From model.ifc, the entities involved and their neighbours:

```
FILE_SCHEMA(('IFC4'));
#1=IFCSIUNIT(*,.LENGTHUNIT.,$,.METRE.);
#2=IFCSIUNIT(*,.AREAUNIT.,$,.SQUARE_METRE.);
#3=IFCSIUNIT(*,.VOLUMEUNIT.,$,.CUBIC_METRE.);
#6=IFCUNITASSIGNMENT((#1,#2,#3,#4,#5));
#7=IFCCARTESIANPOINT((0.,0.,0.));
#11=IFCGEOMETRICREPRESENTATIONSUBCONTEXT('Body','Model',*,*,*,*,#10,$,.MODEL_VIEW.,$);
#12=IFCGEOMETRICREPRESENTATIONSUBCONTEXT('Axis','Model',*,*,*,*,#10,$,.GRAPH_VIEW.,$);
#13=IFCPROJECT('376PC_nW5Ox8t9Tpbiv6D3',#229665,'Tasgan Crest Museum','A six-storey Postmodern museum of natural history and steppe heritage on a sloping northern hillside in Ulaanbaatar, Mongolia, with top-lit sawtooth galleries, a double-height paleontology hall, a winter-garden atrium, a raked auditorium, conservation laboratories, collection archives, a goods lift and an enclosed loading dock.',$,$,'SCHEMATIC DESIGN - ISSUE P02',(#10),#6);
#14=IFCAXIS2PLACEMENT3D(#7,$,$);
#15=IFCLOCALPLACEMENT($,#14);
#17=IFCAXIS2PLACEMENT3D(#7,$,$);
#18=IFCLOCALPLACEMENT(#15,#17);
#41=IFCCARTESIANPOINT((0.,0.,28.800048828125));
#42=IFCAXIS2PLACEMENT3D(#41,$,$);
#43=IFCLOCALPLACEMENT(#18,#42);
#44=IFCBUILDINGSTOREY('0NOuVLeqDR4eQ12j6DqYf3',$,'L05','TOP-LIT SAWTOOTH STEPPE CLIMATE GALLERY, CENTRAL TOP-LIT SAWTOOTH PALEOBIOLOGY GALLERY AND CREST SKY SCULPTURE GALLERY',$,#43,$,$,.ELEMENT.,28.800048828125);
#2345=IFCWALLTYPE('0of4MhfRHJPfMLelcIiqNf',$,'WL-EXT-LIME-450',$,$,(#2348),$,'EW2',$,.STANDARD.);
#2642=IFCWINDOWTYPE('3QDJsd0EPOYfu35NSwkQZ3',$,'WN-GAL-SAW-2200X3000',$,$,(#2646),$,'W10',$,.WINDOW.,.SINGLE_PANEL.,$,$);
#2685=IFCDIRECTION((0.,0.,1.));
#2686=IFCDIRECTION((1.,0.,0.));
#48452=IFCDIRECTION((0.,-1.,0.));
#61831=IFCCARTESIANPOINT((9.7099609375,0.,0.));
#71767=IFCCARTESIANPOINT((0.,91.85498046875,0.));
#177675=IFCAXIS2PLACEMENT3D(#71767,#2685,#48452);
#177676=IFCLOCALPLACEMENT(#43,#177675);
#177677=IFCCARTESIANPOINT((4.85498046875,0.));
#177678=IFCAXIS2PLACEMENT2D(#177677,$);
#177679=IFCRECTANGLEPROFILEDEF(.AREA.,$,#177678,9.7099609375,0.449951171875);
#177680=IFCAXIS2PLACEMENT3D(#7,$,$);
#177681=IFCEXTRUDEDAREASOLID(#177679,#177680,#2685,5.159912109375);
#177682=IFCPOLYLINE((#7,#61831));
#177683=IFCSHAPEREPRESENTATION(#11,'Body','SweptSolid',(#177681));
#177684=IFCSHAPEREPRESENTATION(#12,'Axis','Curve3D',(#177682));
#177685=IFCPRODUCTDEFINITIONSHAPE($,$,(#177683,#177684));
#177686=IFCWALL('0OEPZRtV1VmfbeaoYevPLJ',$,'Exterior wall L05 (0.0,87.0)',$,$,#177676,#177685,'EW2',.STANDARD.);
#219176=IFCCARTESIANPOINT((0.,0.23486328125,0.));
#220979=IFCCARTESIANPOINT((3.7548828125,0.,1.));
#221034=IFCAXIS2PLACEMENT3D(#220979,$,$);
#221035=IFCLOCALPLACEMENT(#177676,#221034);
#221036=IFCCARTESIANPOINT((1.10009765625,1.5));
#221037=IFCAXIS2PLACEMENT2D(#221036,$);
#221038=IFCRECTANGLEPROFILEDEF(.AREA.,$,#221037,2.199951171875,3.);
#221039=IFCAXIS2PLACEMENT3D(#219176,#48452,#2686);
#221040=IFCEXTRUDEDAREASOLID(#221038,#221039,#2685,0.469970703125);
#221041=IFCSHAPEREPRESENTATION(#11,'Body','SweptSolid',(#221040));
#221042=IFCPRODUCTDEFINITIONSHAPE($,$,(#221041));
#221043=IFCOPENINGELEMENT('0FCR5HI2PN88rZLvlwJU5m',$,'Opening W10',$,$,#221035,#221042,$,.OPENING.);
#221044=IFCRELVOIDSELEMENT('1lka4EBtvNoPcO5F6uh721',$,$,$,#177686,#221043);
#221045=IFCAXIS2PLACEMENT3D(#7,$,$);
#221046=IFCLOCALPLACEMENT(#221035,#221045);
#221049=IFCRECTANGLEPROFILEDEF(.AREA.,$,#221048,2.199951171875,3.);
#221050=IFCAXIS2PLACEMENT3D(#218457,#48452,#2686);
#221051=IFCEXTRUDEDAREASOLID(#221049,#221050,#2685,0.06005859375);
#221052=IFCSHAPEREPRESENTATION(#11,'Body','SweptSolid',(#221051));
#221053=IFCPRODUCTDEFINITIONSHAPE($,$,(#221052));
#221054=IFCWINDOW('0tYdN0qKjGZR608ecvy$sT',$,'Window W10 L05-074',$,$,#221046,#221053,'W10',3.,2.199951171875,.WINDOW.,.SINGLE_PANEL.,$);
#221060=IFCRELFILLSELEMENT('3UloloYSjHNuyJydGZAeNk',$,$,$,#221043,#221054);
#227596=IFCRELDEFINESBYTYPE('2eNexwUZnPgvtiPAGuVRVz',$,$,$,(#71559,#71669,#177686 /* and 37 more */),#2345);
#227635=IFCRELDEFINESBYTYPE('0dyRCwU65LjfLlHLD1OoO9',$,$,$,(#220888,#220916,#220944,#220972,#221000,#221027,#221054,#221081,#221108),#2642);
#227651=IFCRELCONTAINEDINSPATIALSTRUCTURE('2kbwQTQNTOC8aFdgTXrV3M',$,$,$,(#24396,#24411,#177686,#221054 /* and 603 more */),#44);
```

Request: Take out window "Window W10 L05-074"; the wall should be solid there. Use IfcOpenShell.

```python
import ifcopenshell
import ifcopenshell.api.feature
import ifcopenshell.api.root
import ifcopenshell.geom
import ifcopenshell.util.shape

model = ifcopenshell.open("model.ifc")
settings = ifcopenshell.geom.settings()


def volume(element):
    """Net volume in cubic metres, openings subtracted."""
    shape = ifcopenshell.geom.create_shape(settings, element)
    return ifcopenshell.util.shape.get_volume(shape.geometry)


window = model.by_id(221054)
opening = window.FillsVoids[0].RelatingOpeningElement
wall = opening.VoidsElements[0].RelatingBuildingElement
before = volume(wall)

ifcopenshell.api.root.remove_product(model, product=window)
ifcopenshell.api.feature.remove_feature(model, feature=opening)

after = volume(wall)

print(f"wall volume {before:.3f} -> {after:.3f} m3")

model.write("model-out.ifc")
```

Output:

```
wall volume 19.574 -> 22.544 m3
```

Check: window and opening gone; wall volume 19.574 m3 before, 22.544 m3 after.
